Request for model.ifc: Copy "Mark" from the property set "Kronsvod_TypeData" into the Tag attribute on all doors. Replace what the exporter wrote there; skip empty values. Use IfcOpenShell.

First a look at what the model holds.

```python
import ifcopenshell
import ifcopenshell.util.element

model = ifcopenshell.open("model.ifc")
print(model.schema)
doors = model.by_type("IfcDoor")
print(len(doors), "doors")
for e in doors[:8]:
    source = ifcopenshell.util.element.get_pset(e, "Kronsvod_TypeData", "Mark")
    target = e.Tag
    print(e.id(), repr(source), repr(target), sep=" | ")
```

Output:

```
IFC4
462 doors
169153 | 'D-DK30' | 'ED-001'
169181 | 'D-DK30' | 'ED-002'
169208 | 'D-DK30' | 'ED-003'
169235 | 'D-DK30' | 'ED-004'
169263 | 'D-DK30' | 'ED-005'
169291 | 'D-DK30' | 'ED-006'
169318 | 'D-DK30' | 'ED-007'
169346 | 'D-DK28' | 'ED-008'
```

```python
import ifcopenshell
import ifcopenshell.util.element

model = ifcopenshell.open("model.ifc")

count = 0
for e in model.by_type("IfcDoor"):
    value = ifcopenshell.util.element.get_pset(e, "Kronsvod_TypeData", "Mark")
    current = e.Tag
    if not value or not value.strip() or current == value:
        continue
    e.Tag = value
    count += 1

print(count, "doors updated")

model.write("model_rev.ifc")
```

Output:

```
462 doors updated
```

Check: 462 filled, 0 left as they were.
